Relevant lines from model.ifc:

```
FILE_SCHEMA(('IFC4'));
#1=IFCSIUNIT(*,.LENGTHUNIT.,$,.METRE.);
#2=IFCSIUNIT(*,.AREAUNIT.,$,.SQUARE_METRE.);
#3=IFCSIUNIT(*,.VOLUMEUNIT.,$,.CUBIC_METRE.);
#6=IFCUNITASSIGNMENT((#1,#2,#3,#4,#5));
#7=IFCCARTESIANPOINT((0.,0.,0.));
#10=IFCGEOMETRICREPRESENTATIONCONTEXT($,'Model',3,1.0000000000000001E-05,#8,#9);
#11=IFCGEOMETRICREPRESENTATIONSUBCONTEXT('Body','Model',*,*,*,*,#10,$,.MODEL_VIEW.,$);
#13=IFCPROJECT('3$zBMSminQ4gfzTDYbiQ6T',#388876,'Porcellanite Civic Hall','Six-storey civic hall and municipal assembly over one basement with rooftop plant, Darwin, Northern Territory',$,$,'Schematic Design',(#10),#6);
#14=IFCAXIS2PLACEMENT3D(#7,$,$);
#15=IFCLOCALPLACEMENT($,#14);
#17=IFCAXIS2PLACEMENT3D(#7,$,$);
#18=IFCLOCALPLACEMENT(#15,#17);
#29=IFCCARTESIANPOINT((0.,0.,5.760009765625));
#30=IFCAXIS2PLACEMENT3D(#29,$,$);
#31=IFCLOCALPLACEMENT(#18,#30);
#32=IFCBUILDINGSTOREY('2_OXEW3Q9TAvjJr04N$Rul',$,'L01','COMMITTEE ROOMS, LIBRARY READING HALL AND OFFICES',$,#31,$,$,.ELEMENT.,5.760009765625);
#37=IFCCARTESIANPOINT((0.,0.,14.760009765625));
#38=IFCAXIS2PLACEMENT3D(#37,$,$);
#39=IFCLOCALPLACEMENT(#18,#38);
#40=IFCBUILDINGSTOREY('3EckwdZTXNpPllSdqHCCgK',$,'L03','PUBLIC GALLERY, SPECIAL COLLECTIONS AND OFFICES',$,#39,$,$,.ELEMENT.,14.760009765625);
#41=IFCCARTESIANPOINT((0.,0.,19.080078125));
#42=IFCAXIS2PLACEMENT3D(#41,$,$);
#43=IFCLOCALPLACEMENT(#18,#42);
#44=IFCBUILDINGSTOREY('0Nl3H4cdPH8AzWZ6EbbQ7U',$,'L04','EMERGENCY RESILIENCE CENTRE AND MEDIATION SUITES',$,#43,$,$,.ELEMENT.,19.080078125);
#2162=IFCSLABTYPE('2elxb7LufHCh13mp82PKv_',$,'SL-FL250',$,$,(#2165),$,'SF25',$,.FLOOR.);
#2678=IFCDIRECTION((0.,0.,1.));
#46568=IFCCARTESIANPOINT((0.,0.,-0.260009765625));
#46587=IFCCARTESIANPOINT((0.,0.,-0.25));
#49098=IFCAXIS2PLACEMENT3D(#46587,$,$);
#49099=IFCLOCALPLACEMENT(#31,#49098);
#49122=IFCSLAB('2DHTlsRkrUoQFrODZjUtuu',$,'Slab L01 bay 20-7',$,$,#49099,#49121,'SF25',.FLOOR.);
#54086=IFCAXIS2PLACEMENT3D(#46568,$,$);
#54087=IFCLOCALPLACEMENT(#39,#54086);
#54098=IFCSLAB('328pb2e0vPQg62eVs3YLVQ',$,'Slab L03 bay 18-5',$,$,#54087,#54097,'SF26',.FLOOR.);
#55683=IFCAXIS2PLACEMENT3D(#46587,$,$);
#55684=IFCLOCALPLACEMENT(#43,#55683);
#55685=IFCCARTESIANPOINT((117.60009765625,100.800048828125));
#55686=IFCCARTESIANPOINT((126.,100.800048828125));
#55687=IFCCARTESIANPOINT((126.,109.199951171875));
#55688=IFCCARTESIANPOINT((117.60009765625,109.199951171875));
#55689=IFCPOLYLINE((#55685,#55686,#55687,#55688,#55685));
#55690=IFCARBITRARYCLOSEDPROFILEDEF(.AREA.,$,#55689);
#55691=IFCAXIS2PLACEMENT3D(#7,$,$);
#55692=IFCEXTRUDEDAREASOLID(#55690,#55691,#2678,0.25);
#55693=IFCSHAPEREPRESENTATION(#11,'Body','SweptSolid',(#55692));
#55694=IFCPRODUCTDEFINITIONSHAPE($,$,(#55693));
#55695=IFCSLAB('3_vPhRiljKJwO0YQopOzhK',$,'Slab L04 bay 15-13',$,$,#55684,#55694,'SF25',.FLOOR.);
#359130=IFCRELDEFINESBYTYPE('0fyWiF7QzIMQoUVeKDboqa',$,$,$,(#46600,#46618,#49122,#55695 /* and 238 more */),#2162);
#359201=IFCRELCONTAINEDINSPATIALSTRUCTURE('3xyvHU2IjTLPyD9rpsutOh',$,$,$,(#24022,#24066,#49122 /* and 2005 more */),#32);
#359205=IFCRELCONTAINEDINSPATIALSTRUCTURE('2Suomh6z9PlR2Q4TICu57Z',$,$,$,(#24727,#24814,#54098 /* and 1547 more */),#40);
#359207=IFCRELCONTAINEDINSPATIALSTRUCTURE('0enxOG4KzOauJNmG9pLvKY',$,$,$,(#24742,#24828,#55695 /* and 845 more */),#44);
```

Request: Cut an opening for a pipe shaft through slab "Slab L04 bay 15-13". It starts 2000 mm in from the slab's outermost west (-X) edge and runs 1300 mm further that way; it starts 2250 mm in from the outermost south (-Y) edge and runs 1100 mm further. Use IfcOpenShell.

```python
import numpy as np
import ifcopenshell
import ifcopenshell.api.feature
import ifcopenshell.api.geometry
import ifcopenshell.api.root
import ifcopenshell.geom
import ifcopenshell.util.placement
import ifcopenshell.util.representation
import ifcopenshell.util.shape
import ifcopenshell.util.unit

model = ifcopenshell.open("model.ifc")
unit_scale = ifcopenshell.util.unit.calculate_unit_scale(model)
settings = ifcopenshell.geom.settings()


def volume(element):
    """Net volume in cubic metres, openings subtracted."""
    shape = ifcopenshell.geom.create_shape(settings, element)
    return ifcopenshell.util.shape.get_volume(shape.geometry)


slab = model.by_guid("3_vPhRiljKJwO0YQopOzhK")
before = volume(slab)

# Extent in the slab's own axes, in metres. The edges named are its -X and -Y sides.
slab_shape = ifcopenshell.geom.create_shape(settings, slab)
vertices = ifcopenshell.util.shape.get_vertices(slab_shape.geometry)
x_min, y_min, bottom = vertices.min(axis=0)
top = vertices[:, 2].max()

opening = ifcopenshell.api.root.create_entity(model, ifc_class="IfcOpeningElement", name="Pipe shaft opening", predefined_type="OPENING")
context = ifcopenshell.util.representation.get_context(model, "Model", "Body", "MODEL_VIEW")
width, depth = 1.3, 1.1
outline = [(0.0, 0.0), (width, 0.0), (width, depth), (0.0, depth), (0.0, 0.0)]
# Overshoot both faces by 50 mm so the cut is clean.
shape = ifcopenshell.api.geometry.add_slab_representation(
    model, context=context, depth=top - bottom + 0.1, polyline=outline
)
ifcopenshell.api.geometry.assign_representation(model, product=opening, representation=shape)

matrix = ifcopenshell.util.placement.get_local_placement(slab.ObjectPlacement)
matrix[:, 3] = matrix @ np.append(np.array([x_min + 2, y_min + 2.25, bottom - 0.05]) / unit_scale, 1.0)
ifcopenshell.api.geometry.edit_object_placement(model, product=opening, matrix=matrix, is_si=False)
ifcopenshell.api.feature.add_feature(model, feature=opening, element=slab)

after = volume(slab)

print(f"slab volume {before:.3f} -> {after:.3f} m3")

model.write("model-out.ifc")
```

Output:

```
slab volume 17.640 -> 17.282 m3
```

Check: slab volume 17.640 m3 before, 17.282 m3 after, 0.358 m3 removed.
